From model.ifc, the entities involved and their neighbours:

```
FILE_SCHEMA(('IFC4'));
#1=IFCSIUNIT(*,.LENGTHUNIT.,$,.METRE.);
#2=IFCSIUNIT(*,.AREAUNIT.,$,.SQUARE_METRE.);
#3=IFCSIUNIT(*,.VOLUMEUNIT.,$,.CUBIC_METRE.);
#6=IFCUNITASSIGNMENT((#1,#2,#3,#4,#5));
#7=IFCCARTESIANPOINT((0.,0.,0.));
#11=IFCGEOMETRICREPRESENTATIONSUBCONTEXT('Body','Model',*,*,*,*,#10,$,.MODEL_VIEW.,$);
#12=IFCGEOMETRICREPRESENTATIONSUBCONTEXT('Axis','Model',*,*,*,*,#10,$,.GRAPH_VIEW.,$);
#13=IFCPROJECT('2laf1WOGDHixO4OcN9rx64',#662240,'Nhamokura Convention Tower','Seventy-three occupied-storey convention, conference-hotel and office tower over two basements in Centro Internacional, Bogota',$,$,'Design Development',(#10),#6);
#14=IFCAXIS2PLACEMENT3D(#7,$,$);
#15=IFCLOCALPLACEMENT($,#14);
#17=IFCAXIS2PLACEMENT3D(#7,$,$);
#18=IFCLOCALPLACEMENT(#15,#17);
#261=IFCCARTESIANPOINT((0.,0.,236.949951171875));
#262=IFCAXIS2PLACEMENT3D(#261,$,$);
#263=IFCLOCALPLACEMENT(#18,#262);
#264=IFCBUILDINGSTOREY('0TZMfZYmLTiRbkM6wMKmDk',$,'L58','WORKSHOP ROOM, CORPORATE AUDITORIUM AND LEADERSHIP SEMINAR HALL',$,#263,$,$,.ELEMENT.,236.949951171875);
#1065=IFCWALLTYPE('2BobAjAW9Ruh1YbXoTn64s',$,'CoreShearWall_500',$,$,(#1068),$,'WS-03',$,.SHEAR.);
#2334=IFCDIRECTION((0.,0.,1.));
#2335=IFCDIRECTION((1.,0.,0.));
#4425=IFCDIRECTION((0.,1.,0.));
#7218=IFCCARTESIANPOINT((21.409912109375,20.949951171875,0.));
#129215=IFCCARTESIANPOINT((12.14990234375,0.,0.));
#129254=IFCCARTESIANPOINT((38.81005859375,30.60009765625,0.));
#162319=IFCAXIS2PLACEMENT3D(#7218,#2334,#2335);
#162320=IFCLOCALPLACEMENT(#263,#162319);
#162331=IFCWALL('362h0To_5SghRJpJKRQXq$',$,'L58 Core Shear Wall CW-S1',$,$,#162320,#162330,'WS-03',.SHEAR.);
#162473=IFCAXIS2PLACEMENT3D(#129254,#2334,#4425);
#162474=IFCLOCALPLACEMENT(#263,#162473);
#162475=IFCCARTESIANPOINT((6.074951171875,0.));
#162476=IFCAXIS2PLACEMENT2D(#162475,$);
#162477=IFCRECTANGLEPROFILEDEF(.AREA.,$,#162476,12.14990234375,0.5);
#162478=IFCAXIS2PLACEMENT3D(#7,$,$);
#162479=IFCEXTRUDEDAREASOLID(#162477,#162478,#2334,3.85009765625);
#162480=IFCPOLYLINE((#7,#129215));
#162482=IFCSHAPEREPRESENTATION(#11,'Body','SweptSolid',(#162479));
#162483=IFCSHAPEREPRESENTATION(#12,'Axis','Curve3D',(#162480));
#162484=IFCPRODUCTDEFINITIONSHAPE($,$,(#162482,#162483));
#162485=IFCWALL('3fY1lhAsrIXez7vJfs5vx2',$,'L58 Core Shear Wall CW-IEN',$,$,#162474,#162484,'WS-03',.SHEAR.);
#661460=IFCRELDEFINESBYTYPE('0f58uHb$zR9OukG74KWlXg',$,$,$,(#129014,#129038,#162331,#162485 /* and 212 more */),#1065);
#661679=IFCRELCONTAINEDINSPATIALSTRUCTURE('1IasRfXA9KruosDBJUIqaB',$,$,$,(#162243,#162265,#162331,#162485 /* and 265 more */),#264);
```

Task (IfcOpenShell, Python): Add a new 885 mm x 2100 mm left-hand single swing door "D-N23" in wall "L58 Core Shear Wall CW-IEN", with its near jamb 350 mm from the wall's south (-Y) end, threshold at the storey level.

```python
import numpy as np
import ifcopenshell
import ifcopenshell.api.feature
import ifcopenshell.api.geometry
import ifcopenshell.api.root
import ifcopenshell.api.spatial
import ifcopenshell.geom
import ifcopenshell.util.element
import ifcopenshell.util.placement
import ifcopenshell.util.representation
import ifcopenshell.util.shape
import ifcopenshell.util.unit

model = ifcopenshell.open("model.ifc")
unit_scale = ifcopenshell.util.unit.calculate_unit_scale(model)
settings = ifcopenshell.geom.settings()


def volume(element):
    """Net volume in cubic metres, openings subtracted."""
    shape = ifcopenshell.geom.create_shape(settings, element)
    return ifcopenshell.util.shape.get_volume(shape.geometry)


wall = model.by_id(162485)
storey = ifcopenshell.util.element.get_container(wall, ifc_class="IfcBuildingStorey")
context = ifcopenshell.util.representation.get_context(model, "Model", "Body", "MODEL_VIEW")
before = volume(wall)

width, height, from_end, sill = 0.885, 2.1, 0.35, 0.0  # metres

# The wall runs along its own X axis, and the end named is its -X end.
wall_shape = ifcopenshell.geom.create_shape(settings, wall)
x, y, z = ifcopenshell.util.shape.get_vertices(wall_shape.geometry).T
start = x.min() + from_end
face, thickness = float(y.min()), float(y.max() - y.min())
wall_matrix = ifcopenshell.util.placement.get_local_placement(wall.ObjectPlacement)
level = ifcopenshell.util.placement.get_local_placement(storey.ObjectPlacement)[2, 3]


def in_wall(x, y):
    """Placement at x, y metres in the wall's axes, at sill height."""
    matrix = wall_matrix.copy()
    matrix[:, 3] = wall_matrix @ np.array([x / unit_scale, y / unit_scale, 0.0, 1.0])
    matrix[2, 3] = level + sill / unit_scale
    return matrix


# Opening: a box that overshoots both wall faces by 50 mm.
opening = ifcopenshell.api.root.create_entity(model, ifc_class="IfcOpeningElement", predefined_type="OPENING")
box = ifcopenshell.api.geometry.add_wall_representation(
    model, context=context, length=width, height=height, thickness=thickness + 0.1
)
ifcopenshell.api.geometry.assign_representation(model, product=opening, representation=box)
ifcopenshell.api.geometry.edit_object_placement(model, product=opening, matrix=in_wall(start, face - 0.05), is_si=False)
ifcopenshell.api.feature.add_feature(model, feature=opening, element=wall)

door = ifcopenshell.api.root.create_entity(model, ifc_class="IfcDoor", name="D-N23", predefined_type="DOOR")
door.OverallWidth, door.OverallHeight = width / unit_scale, height / unit_scale
door.OperationType = "SINGLE_SWING_LEFT"
body = ifcopenshell.api.geometry.add_door_representation(
    model,
    context=context,
    overall_width=door.OverallWidth,
    overall_height=door.OverallHeight,
    operation_type="SINGLE_SWING_LEFT",
    lining_properties={"LiningDepth": thickness / unit_scale, "ThresholdDepth": thickness / unit_scale},
)
ifcopenshell.api.geometry.assign_representation(model, product=door, representation=body)
ifcopenshell.api.spatial.assign_container(model, products=[door], relating_structure=storey)
ifcopenshell.api.feature.add_filling(model, opening=opening, element=door)

# The lining spans the wall, so the door starts at the wall face.
ifcopenshell.api.geometry.edit_object_placement(model, product=door, matrix=in_wall(start, face), is_si=False)

after = volume(wall)

print(f"wall volume {before:.3f} -> {after:.3f} m3")

model.write("model-out.ifc")
```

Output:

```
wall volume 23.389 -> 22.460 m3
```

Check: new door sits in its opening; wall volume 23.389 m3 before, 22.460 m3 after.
